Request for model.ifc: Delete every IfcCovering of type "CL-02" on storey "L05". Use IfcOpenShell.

First a look at what the model holds.

```python
import ifcopenshell
import ifcopenshell.util.element

model = ifcopenshell.open("model.ifc")
print(model.schema)
storey = next(s for s in model.by_type("IfcBuildingStorey") if s.Name == "L05")
coverings = [e for e in ifcopenshell.util.element.get_decomposition(storey) if e.is_a("IfcCovering")]
seen = {}
for e in coverings:
    element_type = ifcopenshell.util.element.get_type(e)
    name = element_type.Name if element_type not in (None, e) else None
    seen[name] = seen.get(name, 0) + 1
for name, count in sorted(seen.items(), key=str):
    print(count, "x", name)
```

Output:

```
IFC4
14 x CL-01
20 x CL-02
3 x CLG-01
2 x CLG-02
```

```python
import ifcopenshell
import ifcopenshell.api.root
import ifcopenshell.util.element

model = ifcopenshell.open("model.ifc")

storey = next(s for s in model.by_type("IfcBuildingStorey") if s.Name == "L05")
coverings = [e for e in ifcopenshell.util.element.get_decomposition(storey) if e.is_a("IfcCovering")]
targets = [e for e in coverings if (t := ifcopenshell.util.element.get_type(e)) not in (None, e) and t.Name == "CL-02"]

for e in targets:
    ifcopenshell.api.root.remove_product(model, product=e)
print(len(targets), "removed")

model.write("model_v2.ifc")
```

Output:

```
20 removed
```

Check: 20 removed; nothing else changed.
